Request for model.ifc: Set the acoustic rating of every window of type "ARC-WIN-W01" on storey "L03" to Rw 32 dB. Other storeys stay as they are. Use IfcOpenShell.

First a look at what the model holds.

```python
import ifcopenshell
import ifcopenshell.util.element

model = ifcopenshell.open("model.ifc")
print(model.schema)
storey = next(s for s in model.by_type("IfcBuildingStorey") if s.Name == "L03")
windows = [e for e in ifcopenshell.util.element.get_decomposition(storey) if e.is_a("IfcWindow")]
seen = {}
for e in windows:
    element_type = ifcopenshell.util.element.get_type(e)
    key = (element_type.Name if element_type != e and element_type else None, ifcopenshell.util.element.get_pset(e, "Pset_WindowCommon", "AcousticRating"))
    seen[key] = seen.get(key, 0) + 1
for (name, value), count in sorted(seen.items(), key=str):
    print(count, "x", name, "|", value)
```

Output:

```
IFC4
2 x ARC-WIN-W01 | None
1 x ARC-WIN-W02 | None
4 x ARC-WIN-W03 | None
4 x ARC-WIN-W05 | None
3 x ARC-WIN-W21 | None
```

```python
import ifcopenshell
import ifcopenshell.api.pset
import ifcopenshell.util.element

model = ifcopenshell.open("model.ifc")

storey = next(s for s in model.by_type("IfcBuildingStorey") if s.Name == "L03")
windows = [e for e in ifcopenshell.util.element.get_decomposition(storey) if e.is_a("IfcWindow")]

count = 0
for e in windows:
    element_type = ifcopenshell.util.element.get_type(e)
    if element_type in (None, e) or element_type.Name != "ARC-WIN-W01":
        continue
    # add_pset returns the element's existing set when there is one.
    pset = ifcopenshell.api.pset.add_pset(model, product=e, name="Pset_WindowCommon")
    ifcopenshell.api.pset.edit_pset(model, pset=pset, properties={"AcousticRating": "Rw 32 dB"})
    count += 1

print(count, "windows updated")

model.write("model_v2.ifc")
```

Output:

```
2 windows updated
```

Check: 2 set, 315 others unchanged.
